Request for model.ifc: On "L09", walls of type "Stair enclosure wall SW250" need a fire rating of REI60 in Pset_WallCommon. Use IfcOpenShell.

First a look at what the model holds.

```python
import ifcopenshell
import ifcopenshell.util.element

model = ifcopenshell.open("model.ifc")
print(model.schema)
storey = next(s for s in model.by_type("IfcBuildingStorey") if s.Name == "L09")
walls = [e for e in ifcopenshell.util.element.get_decomposition(storey) if e.is_a("IfcWall")]
seen = {}
for e in walls:
    element_type = ifcopenshell.util.element.get_type(e)
    key = (element_type.Name if element_type != e and element_type else None, ifcopenshell.util.element.get_pset(e, "Pset_WallCommon", "FireRating"))
    seen[key] = seen.get(key, 0) + 1
for (name, value), count in sorted(seen.items(), key=str):
    print(count, "x", name, "|", value)
```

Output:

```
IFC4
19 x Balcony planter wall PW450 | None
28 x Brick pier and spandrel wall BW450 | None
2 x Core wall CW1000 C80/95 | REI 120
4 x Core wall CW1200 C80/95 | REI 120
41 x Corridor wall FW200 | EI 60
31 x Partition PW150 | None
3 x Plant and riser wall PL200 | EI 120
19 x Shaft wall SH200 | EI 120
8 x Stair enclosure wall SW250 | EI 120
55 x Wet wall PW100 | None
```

```python
import ifcopenshell
import ifcopenshell.api.pset
import ifcopenshell.util.element

model = ifcopenshell.open("model.ifc")

storey = next(s for s in model.by_type("IfcBuildingStorey") if s.Name == "L09")
walls = [e for e in ifcopenshell.util.element.get_decomposition(storey) if e.is_a("IfcWall")]

count = 0
for e in walls:
    element_type = ifcopenshell.util.element.get_type(e)
    if element_type in (None, e) or element_type.Name != "Stair enclosure wall SW250":
        continue
    found = ifcopenshell.util.element.get_pset(e, "Pset_WallCommon", should_inherit=False)
    if found:
        pset = model.by_id(found["id"])
        if len(ifcopenshell.util.element.get_elements_by_pset(pset)) > 1:
            pset = ifcopenshell.api.pset.unshare_pset(model, products=[e], pset=pset)[0]
    else:
        pset = ifcopenshell.api.pset.add_pset(model, product=e, name="Pset_WallCommon")
    ifcopenshell.api.pset.edit_pset(model, pset=pset, properties={"FireRating": "REI60"})
    count += 1

print(count, "walls updated")

model.write("model_v2.ifc")
```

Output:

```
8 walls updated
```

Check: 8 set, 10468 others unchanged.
